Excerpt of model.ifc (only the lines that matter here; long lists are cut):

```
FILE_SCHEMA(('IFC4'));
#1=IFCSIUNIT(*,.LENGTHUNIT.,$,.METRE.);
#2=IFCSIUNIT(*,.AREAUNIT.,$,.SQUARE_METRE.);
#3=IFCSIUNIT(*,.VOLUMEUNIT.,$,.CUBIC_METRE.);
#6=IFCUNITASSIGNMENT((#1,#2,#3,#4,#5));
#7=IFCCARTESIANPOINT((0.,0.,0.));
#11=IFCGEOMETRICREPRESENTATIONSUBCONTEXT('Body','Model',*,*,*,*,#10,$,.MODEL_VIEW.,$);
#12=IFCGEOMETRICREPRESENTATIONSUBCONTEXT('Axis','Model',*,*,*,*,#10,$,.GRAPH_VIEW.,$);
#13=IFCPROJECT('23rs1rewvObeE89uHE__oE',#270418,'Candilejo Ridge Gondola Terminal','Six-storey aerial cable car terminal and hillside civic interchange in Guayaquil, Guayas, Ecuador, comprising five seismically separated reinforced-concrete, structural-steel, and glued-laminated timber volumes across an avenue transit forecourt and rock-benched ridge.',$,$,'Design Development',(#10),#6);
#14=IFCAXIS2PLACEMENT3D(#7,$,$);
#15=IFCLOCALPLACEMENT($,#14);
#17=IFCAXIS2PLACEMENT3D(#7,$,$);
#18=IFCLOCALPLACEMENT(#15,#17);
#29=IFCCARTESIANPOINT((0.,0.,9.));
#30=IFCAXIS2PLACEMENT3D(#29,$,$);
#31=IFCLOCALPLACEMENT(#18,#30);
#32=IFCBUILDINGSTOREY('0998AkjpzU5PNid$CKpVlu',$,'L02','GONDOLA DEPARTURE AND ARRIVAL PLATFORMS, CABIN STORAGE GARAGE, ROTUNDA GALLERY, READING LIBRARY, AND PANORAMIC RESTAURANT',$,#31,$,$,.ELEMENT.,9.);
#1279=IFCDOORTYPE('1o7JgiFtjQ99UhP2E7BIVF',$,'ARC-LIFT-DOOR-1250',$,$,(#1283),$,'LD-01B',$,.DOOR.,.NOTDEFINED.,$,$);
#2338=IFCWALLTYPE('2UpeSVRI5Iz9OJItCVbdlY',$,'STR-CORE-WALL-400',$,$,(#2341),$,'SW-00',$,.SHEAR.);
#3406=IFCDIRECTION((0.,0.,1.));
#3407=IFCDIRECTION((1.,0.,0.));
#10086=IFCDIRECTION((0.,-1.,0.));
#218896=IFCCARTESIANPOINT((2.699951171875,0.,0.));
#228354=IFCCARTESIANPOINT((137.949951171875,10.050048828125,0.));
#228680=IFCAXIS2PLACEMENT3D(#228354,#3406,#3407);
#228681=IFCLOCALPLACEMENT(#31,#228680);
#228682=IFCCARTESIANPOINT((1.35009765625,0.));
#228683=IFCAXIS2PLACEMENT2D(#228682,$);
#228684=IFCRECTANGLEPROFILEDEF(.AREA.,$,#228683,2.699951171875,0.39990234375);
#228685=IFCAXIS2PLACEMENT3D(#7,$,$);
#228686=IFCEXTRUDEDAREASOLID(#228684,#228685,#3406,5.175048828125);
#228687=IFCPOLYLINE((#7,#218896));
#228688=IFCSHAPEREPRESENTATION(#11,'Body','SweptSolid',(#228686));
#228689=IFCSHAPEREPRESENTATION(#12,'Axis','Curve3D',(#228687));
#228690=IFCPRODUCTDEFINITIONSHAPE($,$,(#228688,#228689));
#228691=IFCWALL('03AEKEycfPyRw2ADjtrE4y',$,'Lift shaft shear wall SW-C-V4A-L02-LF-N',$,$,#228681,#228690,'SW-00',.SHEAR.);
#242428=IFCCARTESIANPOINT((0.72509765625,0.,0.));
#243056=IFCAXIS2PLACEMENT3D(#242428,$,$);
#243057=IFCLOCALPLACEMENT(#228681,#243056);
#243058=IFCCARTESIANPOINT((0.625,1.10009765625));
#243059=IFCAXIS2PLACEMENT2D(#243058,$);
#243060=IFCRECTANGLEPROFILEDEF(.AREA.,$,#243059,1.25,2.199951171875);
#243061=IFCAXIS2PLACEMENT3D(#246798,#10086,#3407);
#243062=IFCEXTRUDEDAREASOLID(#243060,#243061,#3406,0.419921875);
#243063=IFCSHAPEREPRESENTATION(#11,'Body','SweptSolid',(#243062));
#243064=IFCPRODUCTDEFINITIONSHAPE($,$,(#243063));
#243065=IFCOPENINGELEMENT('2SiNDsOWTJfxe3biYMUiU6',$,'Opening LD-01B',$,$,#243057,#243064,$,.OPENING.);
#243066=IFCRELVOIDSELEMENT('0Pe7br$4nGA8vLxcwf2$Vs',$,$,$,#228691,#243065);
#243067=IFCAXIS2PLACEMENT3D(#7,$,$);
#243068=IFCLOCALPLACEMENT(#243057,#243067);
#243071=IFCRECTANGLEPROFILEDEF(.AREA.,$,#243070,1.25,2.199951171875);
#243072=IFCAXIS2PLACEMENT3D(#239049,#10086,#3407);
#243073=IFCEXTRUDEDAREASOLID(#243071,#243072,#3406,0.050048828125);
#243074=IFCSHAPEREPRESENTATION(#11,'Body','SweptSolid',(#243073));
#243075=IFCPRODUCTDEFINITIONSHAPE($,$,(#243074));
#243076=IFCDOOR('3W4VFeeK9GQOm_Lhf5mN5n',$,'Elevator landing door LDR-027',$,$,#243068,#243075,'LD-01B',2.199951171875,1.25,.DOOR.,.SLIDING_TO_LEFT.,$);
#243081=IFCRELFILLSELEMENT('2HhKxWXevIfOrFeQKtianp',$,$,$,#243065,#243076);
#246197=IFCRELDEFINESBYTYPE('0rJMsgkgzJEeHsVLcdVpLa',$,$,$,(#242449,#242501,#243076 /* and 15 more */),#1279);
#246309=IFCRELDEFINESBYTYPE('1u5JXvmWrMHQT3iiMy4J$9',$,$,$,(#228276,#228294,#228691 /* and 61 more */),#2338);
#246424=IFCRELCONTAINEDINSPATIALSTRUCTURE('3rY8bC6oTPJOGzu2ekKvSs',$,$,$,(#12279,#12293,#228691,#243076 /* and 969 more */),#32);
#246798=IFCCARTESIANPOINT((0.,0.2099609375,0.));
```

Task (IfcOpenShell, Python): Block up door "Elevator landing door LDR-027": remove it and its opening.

```python
import ifcopenshell
import ifcopenshell.api.feature
import ifcopenshell.api.root
import ifcopenshell.geom
import ifcopenshell.util.shape

model = ifcopenshell.open("model.ifc")
settings = ifcopenshell.geom.settings()


def volume(element):
    """Net volume in cubic metres, openings subtracted."""
    shape = ifcopenshell.geom.create_shape(settings, element)
    return ifcopenshell.util.shape.get_volume(shape.geometry)


door = model.by_guid("3W4VFeeK9GQOm_Lhf5mN5n")
opening = door.FillsVoids[0].RelatingOpeningElement
wall = opening.VoidsElements[0].RelatingBuildingElement
before = volume(wall)

ifcopenshell.api.root.remove_product(model, product=door)
ifcopenshell.api.feature.remove_feature(model, feature=opening)

after = volume(wall)

print(f"wall volume {before:.3f} -> {after:.3f} m3")

model.write("model_rev.ifc")
```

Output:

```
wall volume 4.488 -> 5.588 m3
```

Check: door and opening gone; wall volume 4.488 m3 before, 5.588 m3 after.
